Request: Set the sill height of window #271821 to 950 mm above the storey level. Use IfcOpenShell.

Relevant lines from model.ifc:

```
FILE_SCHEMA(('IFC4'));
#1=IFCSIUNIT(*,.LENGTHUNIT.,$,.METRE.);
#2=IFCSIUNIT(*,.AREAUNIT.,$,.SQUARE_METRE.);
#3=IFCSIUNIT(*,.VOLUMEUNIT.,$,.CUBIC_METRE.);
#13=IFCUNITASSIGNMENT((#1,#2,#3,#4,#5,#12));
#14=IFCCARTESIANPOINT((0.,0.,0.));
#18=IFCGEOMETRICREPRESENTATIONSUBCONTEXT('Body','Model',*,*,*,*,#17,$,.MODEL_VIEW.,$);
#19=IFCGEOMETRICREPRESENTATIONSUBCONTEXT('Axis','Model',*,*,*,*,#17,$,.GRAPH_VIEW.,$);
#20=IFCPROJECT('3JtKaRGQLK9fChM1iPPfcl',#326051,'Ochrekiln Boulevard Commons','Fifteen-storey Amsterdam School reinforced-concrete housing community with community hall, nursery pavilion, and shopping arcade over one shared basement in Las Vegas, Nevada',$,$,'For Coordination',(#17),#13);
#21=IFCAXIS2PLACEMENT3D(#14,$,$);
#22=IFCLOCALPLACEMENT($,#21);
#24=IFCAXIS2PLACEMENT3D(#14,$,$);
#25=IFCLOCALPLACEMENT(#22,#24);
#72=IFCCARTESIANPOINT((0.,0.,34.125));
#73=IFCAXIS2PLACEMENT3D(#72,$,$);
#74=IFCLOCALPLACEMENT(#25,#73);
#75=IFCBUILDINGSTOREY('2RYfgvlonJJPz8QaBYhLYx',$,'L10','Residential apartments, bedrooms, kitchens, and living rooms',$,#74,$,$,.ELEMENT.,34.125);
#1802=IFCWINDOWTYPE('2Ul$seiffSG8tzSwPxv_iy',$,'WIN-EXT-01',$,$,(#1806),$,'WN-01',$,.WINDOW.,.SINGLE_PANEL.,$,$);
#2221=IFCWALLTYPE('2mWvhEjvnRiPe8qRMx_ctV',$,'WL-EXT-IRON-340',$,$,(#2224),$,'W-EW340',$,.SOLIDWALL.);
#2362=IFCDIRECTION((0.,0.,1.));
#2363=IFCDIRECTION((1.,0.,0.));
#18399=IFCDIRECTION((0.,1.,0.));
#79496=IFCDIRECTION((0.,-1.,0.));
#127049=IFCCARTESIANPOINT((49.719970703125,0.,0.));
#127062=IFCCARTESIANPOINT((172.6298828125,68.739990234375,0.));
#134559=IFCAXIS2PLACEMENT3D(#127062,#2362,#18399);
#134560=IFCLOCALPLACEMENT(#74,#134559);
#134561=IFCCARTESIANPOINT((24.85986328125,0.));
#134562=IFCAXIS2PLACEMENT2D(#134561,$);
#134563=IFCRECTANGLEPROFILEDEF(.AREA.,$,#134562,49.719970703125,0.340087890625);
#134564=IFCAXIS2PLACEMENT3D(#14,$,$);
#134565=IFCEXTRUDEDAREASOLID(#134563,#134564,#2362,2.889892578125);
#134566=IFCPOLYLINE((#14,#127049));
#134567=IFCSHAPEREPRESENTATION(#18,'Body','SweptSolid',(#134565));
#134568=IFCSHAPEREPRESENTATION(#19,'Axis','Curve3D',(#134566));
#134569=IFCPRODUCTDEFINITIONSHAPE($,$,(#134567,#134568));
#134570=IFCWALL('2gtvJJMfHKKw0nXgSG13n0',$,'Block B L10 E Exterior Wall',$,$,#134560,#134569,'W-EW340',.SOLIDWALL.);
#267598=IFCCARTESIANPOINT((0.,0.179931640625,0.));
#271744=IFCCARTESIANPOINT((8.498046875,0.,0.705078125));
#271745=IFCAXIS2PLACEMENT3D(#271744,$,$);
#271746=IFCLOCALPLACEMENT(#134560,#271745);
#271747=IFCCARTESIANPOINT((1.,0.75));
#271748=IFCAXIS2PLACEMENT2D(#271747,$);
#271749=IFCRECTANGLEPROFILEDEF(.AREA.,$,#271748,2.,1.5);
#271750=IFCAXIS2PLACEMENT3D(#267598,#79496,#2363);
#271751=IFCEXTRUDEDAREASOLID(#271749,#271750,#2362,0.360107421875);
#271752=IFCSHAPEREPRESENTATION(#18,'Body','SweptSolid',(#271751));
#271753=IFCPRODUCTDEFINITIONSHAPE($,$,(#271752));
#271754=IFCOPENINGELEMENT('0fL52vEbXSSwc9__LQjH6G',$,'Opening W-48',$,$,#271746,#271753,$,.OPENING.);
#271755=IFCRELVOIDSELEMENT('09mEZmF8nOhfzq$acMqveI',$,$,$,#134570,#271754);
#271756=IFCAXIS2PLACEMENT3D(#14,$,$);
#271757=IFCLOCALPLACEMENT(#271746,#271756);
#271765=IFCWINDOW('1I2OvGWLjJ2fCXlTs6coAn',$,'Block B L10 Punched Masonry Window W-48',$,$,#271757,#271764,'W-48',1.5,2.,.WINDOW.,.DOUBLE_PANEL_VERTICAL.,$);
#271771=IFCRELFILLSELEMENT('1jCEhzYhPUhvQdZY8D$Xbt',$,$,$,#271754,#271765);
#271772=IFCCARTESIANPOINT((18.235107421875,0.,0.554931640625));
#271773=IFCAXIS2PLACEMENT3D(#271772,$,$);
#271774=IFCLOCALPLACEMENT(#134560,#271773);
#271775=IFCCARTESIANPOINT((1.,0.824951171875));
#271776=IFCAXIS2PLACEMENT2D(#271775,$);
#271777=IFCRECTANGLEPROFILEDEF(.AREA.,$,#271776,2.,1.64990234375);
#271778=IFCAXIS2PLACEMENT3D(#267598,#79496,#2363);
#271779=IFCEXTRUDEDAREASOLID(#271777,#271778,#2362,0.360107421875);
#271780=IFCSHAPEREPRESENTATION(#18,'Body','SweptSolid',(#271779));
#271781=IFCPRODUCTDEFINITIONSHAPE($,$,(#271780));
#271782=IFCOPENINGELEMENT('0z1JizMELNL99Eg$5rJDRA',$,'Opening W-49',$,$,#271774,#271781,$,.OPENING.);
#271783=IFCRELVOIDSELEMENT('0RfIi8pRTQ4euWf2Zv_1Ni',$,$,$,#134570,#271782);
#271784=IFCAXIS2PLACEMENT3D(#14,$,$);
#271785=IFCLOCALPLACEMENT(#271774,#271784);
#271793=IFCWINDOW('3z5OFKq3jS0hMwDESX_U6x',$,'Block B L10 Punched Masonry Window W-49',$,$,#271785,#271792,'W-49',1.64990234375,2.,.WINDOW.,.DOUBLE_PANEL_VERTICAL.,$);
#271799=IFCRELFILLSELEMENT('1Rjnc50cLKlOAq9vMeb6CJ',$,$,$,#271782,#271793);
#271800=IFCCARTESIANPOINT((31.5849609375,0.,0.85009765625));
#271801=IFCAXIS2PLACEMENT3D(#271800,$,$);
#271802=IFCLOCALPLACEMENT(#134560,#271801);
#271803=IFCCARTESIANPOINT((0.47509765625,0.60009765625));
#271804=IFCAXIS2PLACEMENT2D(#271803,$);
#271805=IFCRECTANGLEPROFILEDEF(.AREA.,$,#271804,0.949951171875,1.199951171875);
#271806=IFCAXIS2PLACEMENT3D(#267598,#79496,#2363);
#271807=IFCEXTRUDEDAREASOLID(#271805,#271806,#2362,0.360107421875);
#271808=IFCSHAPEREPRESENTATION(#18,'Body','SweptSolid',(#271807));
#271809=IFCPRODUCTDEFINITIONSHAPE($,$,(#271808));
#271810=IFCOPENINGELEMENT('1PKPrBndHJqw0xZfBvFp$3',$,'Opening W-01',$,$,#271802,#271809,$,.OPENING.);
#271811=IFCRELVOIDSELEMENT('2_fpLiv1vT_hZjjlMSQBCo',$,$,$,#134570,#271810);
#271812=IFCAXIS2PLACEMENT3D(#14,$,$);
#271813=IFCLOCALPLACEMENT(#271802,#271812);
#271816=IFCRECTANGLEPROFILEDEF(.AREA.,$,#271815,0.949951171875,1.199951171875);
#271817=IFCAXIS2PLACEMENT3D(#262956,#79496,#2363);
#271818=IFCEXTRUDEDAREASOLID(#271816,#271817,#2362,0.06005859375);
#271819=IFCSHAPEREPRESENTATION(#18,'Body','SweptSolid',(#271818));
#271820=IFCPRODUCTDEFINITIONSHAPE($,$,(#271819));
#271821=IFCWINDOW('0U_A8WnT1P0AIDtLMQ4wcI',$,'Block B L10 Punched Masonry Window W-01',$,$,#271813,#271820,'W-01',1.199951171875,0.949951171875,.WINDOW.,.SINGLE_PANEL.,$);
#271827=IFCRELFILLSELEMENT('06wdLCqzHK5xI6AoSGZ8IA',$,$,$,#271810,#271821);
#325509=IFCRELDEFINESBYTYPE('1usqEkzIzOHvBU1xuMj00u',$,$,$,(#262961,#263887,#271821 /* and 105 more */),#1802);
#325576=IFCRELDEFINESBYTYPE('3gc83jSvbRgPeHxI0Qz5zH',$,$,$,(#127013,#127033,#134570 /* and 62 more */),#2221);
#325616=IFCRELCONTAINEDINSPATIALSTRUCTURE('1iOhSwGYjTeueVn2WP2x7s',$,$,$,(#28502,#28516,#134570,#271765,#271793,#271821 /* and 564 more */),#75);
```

```python
import numpy as np
import ifcopenshell
import ifcopenshell.api.geometry
import ifcopenshell.geom
import ifcopenshell.util.element
import ifcopenshell.util.placement
import ifcopenshell.util.shape
import ifcopenshell.util.unit

model = ifcopenshell.open("model.ifc")
unit_scale = ifcopenshell.util.unit.calculate_unit_scale(model)

window = model.by_guid("0U_A8WnT1P0AIDtLMQ4wcI")
opening = window.FillsVoids[0].RelatingOpeningElement
storey = ifcopenshell.util.element.get_container(window, ifc_class="IfcBuildingStorey")
level = ifcopenshell.util.placement.get_local_placement(storey.ObjectPlacement)[2, 3]

# The opening's origin need not be at the sill, so measure its lowest point.
shape = ifcopenshell.geom.create_shape(ifcopenshell.geom.settings(), opening)
bottom = ifcopenshell.util.shape.get_shape_bottom_elevation(shape, shape.geometry) / unit_scale
dz = level + 0.95 / unit_scale - bottom

shift = np.array([0.0, 0.0, dz])
# The window is placed relative to its opening, so it follows when the opening moves.
matrix = ifcopenshell.util.placement.get_local_placement(opening.ObjectPlacement)
matrix[:3, 3] += shift
ifcopenshell.api.geometry.edit_object_placement(
    model, product=opening, matrix=matrix, is_si=False, should_transform_children=True
)

print(f"moved by {dz * unit_scale:+.3f} m")

model.write("model_rev.ifc")
```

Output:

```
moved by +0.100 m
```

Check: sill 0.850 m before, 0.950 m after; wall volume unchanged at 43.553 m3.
